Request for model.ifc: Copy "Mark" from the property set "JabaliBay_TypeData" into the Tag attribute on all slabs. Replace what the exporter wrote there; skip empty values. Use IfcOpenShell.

First a look at what the model holds.

```python
import ifcopenshell
import ifcopenshell.util.element

model = ifcopenshell.open("model.ifc")
print(model.schema)
slabs = model.by_type("IfcSlab")
print(len(slabs), "slabs")
for e in slabs[:8]:
    source = ifcopenshell.util.element.get_pset(e, "JabaliBay_TypeData", "Mark")
    target = e.Tag
    print(e.id(), repr(source), repr(target), sep=" | ")
```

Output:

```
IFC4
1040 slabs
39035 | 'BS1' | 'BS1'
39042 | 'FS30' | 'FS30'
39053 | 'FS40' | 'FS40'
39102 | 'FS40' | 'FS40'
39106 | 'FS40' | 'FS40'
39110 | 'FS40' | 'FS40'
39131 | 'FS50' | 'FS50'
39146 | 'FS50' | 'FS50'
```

```python
import ifcopenshell
import ifcopenshell.util.element

model = ifcopenshell.open("model.ifc")

count = 0
for e in model.by_type("IfcSlab"):
    value = ifcopenshell.util.element.get_pset(e, "JabaliBay_TypeData", "Mark")
    current = e.Tag
    if not value or not value.strip() or current == value:
        continue
    e.Tag = value
    count += 1

print(count, "slabs updated")

model.write("model_v2.ifc")
```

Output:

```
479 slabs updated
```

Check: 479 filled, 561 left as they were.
